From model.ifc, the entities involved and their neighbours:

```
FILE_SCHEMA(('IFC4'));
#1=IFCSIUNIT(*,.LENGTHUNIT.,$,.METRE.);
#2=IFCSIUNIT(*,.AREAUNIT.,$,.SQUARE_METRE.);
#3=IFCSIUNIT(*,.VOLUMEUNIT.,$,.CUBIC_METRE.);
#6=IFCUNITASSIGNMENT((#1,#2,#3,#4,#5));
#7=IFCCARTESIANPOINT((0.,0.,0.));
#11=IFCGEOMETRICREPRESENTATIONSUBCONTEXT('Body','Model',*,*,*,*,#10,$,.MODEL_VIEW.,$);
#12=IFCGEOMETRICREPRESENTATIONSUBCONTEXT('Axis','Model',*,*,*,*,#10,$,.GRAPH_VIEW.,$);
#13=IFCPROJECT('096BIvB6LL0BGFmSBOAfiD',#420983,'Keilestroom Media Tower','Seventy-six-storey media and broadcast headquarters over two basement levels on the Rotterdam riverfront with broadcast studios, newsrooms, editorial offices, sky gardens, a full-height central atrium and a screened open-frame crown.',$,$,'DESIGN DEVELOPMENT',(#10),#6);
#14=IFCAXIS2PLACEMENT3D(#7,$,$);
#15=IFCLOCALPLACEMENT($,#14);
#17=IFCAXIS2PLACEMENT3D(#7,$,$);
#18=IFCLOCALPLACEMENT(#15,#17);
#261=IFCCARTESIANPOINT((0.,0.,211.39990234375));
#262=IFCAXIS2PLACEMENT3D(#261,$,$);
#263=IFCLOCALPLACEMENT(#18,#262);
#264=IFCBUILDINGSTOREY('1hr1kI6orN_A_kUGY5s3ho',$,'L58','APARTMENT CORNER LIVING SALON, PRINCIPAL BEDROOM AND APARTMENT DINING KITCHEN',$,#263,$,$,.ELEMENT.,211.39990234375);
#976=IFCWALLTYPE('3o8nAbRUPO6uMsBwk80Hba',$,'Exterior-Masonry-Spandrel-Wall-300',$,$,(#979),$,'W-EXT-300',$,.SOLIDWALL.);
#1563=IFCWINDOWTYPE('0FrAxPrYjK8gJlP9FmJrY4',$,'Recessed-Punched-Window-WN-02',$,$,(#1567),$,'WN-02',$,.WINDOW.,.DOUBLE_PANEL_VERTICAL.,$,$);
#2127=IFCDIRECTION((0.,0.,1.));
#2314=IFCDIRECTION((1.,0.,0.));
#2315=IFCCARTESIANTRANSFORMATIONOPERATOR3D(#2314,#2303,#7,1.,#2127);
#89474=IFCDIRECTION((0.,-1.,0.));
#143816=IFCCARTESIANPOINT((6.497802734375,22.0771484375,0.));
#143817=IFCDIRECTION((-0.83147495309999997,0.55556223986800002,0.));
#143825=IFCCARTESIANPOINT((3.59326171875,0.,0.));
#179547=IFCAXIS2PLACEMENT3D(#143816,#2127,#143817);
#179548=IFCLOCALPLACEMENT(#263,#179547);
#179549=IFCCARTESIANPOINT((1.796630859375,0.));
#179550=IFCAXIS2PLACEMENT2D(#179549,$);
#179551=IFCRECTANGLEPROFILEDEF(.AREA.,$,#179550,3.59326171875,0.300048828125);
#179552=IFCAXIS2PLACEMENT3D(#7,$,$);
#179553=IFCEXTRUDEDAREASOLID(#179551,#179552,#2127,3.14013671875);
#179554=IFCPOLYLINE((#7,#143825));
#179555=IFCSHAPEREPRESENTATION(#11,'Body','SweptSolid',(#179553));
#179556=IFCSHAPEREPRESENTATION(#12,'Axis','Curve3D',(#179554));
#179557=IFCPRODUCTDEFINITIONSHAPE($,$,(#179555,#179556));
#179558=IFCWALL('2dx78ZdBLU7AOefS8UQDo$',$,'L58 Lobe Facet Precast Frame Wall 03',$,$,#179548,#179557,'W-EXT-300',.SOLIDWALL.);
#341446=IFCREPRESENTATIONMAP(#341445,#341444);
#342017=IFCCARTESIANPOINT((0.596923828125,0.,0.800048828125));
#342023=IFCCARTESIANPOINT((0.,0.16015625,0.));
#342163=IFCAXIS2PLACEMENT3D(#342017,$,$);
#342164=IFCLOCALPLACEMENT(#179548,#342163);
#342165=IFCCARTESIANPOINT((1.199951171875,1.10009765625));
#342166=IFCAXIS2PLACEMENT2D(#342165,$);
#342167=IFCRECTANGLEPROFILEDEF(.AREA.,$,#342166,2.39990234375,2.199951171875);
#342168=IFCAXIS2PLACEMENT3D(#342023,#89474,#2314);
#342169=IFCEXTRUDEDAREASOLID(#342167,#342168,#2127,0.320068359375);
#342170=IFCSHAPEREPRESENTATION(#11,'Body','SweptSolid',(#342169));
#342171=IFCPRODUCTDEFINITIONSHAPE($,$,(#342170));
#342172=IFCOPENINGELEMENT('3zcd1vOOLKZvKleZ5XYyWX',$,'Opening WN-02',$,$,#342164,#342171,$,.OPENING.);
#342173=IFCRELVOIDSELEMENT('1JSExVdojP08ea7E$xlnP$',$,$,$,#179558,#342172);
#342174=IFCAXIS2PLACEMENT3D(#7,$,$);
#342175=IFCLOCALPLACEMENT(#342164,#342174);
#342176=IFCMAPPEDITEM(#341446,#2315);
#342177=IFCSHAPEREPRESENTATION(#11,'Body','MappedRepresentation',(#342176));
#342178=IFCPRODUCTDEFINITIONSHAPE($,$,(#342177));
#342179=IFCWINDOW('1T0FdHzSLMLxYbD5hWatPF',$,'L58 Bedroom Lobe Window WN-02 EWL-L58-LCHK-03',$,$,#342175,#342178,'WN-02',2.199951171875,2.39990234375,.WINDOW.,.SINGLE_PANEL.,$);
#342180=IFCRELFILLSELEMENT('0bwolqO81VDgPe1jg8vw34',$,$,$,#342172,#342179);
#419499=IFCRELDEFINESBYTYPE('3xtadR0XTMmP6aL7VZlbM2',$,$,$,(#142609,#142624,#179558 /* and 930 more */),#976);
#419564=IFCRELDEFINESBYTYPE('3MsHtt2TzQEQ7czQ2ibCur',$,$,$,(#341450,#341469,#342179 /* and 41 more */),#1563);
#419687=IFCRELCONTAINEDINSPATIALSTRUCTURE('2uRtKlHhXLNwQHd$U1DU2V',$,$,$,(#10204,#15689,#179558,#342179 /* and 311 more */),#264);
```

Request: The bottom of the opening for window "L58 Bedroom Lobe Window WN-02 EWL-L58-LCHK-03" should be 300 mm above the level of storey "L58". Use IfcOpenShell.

```python
import numpy as np
import ifcopenshell
import ifcopenshell.api.geometry
import ifcopenshell.geom
import ifcopenshell.util.element
import ifcopenshell.util.placement
import ifcopenshell.util.shape
import ifcopenshell.util.unit

model = ifcopenshell.open("model.ifc")
unit_scale = ifcopenshell.util.unit.calculate_unit_scale(model)

window = model.by_guid("1T0FdHzSLMLxYbD5hWatPF")
opening = window.FillsVoids[0].RelatingOpeningElement
storey = ifcopenshell.util.element.get_container(window, ifc_class="IfcBuildingStorey")
level = ifcopenshell.util.placement.get_local_placement(storey.ObjectPlacement)[2, 3]

# The opening's origin need not be at the sill, so measure its lowest point.
shape = ifcopenshell.geom.create_shape(ifcopenshell.geom.settings(), opening)
bottom = ifcopenshell.util.shape.get_shape_bottom_elevation(shape, shape.geometry) / unit_scale
dz = level + 0.3 - bottom

shift = np.array([0.0, 0.0, dz])
# The window is placed relative to its opening, so it follows when the opening moves.
matrix = ifcopenshell.util.placement.get_local_placement(opening.ObjectPlacement)
matrix[:3, 3] += shift
ifcopenshell.api.geometry.edit_object_placement(
    model, product=opening, matrix=matrix, is_si=False, should_transform_children=True
)

print(f"moved by {dz * unit_scale:+.3f} m")

model.write("model_updated.ifc")
```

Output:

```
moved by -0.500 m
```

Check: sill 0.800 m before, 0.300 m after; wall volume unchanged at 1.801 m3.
